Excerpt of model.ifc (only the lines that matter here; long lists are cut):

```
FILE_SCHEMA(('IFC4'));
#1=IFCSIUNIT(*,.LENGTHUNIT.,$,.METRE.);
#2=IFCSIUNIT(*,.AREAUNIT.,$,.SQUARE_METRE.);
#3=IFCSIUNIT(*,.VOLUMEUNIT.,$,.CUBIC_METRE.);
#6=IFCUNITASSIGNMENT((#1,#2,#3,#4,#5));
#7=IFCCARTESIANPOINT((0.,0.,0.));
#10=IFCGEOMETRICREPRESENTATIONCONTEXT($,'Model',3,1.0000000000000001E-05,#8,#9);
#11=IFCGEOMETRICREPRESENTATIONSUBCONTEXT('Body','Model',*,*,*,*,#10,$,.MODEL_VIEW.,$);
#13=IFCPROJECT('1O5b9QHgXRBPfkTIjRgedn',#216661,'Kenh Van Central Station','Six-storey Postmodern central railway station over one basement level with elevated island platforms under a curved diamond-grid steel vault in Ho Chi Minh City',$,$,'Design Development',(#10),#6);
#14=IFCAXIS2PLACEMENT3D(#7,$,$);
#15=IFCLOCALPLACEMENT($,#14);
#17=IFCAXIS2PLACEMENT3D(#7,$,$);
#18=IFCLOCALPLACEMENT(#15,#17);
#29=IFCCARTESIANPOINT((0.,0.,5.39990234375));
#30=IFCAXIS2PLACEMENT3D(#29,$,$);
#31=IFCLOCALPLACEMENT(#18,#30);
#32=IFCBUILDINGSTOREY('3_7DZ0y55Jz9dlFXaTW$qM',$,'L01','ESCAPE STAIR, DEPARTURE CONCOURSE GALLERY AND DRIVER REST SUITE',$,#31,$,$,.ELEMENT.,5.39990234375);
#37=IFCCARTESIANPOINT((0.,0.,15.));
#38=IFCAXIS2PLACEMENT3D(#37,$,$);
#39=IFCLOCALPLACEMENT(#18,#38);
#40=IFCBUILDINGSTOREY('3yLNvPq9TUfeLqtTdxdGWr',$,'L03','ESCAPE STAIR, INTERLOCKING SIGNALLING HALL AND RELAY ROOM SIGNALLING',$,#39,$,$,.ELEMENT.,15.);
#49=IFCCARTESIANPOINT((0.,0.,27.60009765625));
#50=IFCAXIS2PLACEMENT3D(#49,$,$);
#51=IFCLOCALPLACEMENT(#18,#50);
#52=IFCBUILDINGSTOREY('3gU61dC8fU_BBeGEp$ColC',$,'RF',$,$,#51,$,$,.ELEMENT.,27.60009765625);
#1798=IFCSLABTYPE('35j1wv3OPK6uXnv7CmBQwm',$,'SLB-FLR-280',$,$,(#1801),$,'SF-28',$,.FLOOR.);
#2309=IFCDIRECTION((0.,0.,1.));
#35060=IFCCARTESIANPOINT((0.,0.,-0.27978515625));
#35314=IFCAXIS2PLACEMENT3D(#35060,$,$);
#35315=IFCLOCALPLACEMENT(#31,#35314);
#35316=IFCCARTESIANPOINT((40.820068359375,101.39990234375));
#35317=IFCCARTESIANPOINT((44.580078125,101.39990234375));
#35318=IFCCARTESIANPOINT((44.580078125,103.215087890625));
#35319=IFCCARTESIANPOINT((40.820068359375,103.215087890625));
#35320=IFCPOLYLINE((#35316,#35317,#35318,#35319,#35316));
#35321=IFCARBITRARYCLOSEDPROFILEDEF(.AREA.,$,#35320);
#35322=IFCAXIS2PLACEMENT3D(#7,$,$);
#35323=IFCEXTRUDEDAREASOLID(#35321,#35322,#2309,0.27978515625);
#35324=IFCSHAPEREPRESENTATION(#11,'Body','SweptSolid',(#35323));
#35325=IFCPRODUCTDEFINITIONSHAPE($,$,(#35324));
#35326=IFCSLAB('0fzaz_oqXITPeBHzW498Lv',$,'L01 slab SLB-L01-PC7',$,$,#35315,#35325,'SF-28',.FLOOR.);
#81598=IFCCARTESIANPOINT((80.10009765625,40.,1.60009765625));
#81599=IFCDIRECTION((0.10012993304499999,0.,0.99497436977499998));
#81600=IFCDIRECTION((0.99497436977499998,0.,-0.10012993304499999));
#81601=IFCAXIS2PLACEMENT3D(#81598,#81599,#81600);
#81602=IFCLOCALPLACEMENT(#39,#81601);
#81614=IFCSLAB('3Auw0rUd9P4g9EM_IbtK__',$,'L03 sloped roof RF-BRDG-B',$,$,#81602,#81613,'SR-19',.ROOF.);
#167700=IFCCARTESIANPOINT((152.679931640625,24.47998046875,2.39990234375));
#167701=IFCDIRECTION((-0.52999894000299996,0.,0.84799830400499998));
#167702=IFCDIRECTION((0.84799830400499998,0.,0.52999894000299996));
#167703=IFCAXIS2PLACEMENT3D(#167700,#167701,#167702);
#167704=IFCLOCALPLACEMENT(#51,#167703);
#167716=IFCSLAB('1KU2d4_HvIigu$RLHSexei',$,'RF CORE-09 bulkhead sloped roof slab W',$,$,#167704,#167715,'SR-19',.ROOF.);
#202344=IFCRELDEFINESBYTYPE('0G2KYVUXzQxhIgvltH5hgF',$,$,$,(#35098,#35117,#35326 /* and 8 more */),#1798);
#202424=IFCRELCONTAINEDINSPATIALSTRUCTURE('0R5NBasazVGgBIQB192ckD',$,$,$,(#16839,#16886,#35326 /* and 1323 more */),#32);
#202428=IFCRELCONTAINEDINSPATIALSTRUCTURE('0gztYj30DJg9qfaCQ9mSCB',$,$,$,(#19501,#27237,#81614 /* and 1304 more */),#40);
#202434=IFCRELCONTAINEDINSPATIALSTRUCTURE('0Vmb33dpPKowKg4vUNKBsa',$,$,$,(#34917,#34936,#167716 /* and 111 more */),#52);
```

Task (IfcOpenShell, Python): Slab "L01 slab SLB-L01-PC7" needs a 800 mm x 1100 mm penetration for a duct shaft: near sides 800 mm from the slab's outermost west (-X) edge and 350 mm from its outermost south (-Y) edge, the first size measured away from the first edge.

```python
import numpy as np
import ifcopenshell
import ifcopenshell.api.feature
import ifcopenshell.api.geometry
import ifcopenshell.api.root
import ifcopenshell.geom
import ifcopenshell.util.placement
import ifcopenshell.util.representation
import ifcopenshell.util.shape
import ifcopenshell.util.unit

model = ifcopenshell.open("model.ifc")
unit_scale = ifcopenshell.util.unit.calculate_unit_scale(model)
settings = ifcopenshell.geom.settings()


def volume(element):
    """Net volume in cubic metres, openings subtracted."""
    shape = ifcopenshell.geom.create_shape(settings, element)
    return ifcopenshell.util.shape.get_volume(shape.geometry)


slab = model.by_id(35326)
before = volume(slab)

# Extent in the slab's own axes, in metres. The edges named are its -X and -Y sides.
slab_shape = ifcopenshell.geom.create_shape(settings, slab)
vertices = ifcopenshell.util.shape.get_vertices(slab_shape.geometry)
x_min, y_min, bottom = vertices.min(axis=0)
top = vertices[:, 2].max()

opening = ifcopenshell.api.root.create_entity(model, ifc_class="IfcOpeningElement", name="Duct shaft opening", predefined_type="OPENING")
context = ifcopenshell.util.representation.get_context(model, "Model", "Body", "MODEL_VIEW")
width, depth = 0.8, 1.1
outline = [(0.0, 0.0), (width, 0.0), (width, depth), (0.0, depth), (0.0, 0.0)]
# Overshoot both faces by 50 mm so the cut is clean.
shape = ifcopenshell.api.geometry.add_slab_representation(
    model, context=context, depth=top - bottom + 0.1, polyline=outline
)
ifcopenshell.api.geometry.assign_representation(model, product=opening, representation=shape)

matrix = ifcopenshell.util.placement.get_local_placement(slab.ObjectPlacement)
matrix[:, 3] = matrix @ np.append(np.array([x_min + 0.8, y_min + 0.35, bottom - 0.05]) / unit_scale, 1.0)
ifcopenshell.api.geometry.edit_object_placement(model, product=opening, matrix=matrix, is_si=False)
ifcopenshell.api.feature.add_feature(model, feature=opening, element=slab)

after = volume(slab)

print(f"slab volume {before:.3f} -> {after:.3f} m3")

model.write("model_v2.ifc")
```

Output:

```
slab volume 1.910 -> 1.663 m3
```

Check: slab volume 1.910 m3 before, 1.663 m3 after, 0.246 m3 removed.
